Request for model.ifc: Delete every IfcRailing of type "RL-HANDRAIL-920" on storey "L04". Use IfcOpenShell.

First a look at what the model holds.

```python
import ifcopenshell
import ifcopenshell.util.element

model = ifcopenshell.open("model.ifc")
print(model.schema)
storey = next(s for s in model.by_type("IfcBuildingStorey") if s.Name == "L04")
railings = [e for e in ifcopenshell.util.element.get_decomposition(storey) if e.is_a("IfcRailing")]
seen = {}
for e in railings:
    element_type = ifcopenshell.util.element.get_type(e)
    name = element_type.Name if element_type not in (None, e) else None
    seen[name] = seen.get(name, 0) + 1
for name, count in sorted(seen.items(), key=str):
    print(count, "x", name)
```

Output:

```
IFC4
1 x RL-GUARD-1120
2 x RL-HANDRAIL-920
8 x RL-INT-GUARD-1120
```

```python
import ifcopenshell
import ifcopenshell.api.root
import ifcopenshell.util.element

model = ifcopenshell.open("model.ifc")

storey = next(s for s in model.by_type("IfcBuildingStorey") if s.Name == "L04")
railings = [e for e in ifcopenshell.util.element.get_decomposition(storey) if e.is_a("IfcRailing")]
targets = [e for e in railings if (t := ifcopenshell.util.element.get_type(e)) not in (None, e) and t.Name == "RL-HANDRAIL-920"]

for e in targets:
    ifcopenshell.api.root.remove_product(model, product=e)
print(len(targets), "removed")

model.write("model_edited.ifc")
```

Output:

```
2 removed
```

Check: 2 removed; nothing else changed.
